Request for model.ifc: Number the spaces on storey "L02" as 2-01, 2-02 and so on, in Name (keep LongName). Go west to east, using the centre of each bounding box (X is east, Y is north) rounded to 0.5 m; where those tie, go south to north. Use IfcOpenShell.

First a look at what the model holds.

```python
import ifcopenshell
import ifcopenshell.util.element
import ifcopenshell.util.placement

model = ifcopenshell.open("model.ifc")
print(model.schema)
storey = next(s for s in model.by_type("IfcBuildingStorey") if s.Name == "L02")
spaces = [e for e in ifcopenshell.util.element.get_decomposition(storey) if e.is_a("IfcSpace")]
for e in sorted(spaces, key=lambda e: e.id()):
    origin = ifcopenshell.util.placement.get_local_placement(e.ObjectPlacement)[:3, 3]
    print(e.id(), e.Name, e.LongName, origin.round(2) + 0.0, sep=" | ")
```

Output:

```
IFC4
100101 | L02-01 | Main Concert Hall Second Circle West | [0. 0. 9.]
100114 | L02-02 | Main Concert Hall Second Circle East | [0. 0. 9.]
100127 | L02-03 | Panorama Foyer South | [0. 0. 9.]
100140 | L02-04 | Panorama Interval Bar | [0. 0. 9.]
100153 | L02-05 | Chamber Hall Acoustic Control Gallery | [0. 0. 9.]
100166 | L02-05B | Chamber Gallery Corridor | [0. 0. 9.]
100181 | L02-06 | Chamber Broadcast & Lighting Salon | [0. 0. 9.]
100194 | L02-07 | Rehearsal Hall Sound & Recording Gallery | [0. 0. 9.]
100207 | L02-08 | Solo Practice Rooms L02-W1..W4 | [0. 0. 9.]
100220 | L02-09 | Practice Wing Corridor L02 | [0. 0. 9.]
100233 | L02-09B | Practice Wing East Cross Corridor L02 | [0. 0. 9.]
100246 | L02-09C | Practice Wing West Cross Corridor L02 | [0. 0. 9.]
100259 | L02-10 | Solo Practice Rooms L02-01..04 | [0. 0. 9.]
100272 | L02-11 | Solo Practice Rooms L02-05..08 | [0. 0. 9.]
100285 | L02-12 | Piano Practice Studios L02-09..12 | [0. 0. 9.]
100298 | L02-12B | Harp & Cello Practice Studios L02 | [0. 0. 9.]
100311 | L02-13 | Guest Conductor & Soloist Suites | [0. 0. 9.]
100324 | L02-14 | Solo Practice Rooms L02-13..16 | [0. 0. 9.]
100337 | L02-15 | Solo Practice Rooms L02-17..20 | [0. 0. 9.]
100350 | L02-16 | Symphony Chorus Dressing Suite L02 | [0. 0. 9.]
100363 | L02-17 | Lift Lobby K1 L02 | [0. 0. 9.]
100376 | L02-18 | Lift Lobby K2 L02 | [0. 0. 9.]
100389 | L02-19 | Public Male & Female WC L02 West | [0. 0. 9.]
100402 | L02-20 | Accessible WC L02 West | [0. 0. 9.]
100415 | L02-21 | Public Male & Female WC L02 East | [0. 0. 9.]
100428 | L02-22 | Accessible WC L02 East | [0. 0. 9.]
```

```python
import ifcopenshell
import ifcopenshell.geom
import ifcopenshell.util.element
import ifcopenshell.util.shape

model = ifcopenshell.open("model.ifc")
settings = ifcopenshell.geom.settings()
settings.set("use-world-coords", True)


def centre(element):
    shape = ifcopenshell.geom.create_shape(settings, element)
    return ifcopenshell.util.shape.get_bbox_centroid(shape.geometry)


storey = next(s for s in model.by_type("IfcBuildingStorey") if s.Name == "L02")
spaces = [e for e in ifcopenshell.util.element.get_decomposition(storey) if e.is_a("IfcSpace")]

# Insertion points can sit at a corner or the storey origin, so sort by the geometry (in metres).
centres = {e: centre(e) for e in spaces}
spaces.sort(key=lambda e: (round(centres[e][0] / 0.5), centres[e][1]))

for i, e in enumerate(spaces, start=1):
    number = f"2-{i:02d}"
    e.Name = number
    print(e.id(), number)

model.write("model_updated.ifc")
```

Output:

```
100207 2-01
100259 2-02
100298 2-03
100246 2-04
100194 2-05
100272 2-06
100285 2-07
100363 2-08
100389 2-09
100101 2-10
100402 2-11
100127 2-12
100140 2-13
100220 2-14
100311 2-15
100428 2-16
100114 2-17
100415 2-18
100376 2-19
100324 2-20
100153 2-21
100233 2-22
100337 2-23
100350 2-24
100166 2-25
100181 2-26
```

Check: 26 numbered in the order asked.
